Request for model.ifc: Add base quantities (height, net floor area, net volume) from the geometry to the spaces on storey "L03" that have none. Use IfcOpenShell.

First a look at what the model holds.

```python
import ifcopenshell
import ifcopenshell.util.element
import ifcopenshell.util.unit

model = ifcopenshell.open("model.ifc")
print(model.schema)
for unit_type in ("LENGTHUNIT", "AREAUNIT", "VOLUMEUNIT"):
    print(unit_type, ifcopenshell.util.unit.calculate_unit_scale(model, unit_type))
storey = next(s for s in model.by_type("IfcBuildingStorey") if s.Name == "L03")
spaces = [e for e in ifcopenshell.util.element.get_decomposition(storey) if e.is_a("IfcSpace")]
for e in sorted(spaces, key=lambda e: e.id()):
    print(e.id(), e.is_a(), e.Name, list(ifcopenshell.util.element.get_psets(e, qtos_only=True)), sep=" | ")
```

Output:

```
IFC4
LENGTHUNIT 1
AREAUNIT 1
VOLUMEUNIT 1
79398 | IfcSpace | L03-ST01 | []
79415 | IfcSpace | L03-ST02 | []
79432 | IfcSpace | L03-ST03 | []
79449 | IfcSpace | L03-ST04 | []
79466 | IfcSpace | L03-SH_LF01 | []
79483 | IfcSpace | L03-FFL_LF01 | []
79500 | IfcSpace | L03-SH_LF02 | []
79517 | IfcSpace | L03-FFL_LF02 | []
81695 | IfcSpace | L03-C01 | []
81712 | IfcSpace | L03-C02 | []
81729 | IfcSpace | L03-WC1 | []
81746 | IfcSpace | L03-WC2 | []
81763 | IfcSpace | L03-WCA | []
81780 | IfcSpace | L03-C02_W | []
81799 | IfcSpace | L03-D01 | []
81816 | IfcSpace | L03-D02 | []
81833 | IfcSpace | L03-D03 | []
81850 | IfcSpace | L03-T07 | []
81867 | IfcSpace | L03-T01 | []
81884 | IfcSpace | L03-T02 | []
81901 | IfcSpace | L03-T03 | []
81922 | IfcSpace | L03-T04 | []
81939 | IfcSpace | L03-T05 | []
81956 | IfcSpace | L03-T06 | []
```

```python
import ifcopenshell
import ifcopenshell.api.pset
import ifcopenshell.geom
import ifcopenshell.util.element
import ifcopenshell.util.shape
import ifcopenshell.util.unit

model = ifcopenshell.open("model.ifc")
unit_scale = ifcopenshell.util.unit.calculate_unit_scale(model)
area_scale = ifcopenshell.util.unit.calculate_unit_scale(model, "AREAUNIT")
volume_scale = ifcopenshell.util.unit.calculate_unit_scale(model, "VOLUMEUNIT")
settings = ifcopenshell.geom.settings()

storey = next(s for s in model.by_type("IfcBuildingStorey") if s.Name == "L03")
spaces = [e for e in ifcopenshell.util.element.get_decomposition(storey) if e.is_a("IfcSpace")]

for e in sorted(spaces, key=lambda e: e.id()):
    if ifcopenshell.util.element.get_psets(e, qtos_only=True, should_inherit=False):
        continue
    # Geometry comes back in metres, in the element's own axes.
    shape = ifcopenshell.geom.create_shape(settings, e)
    values = {
        "Height": ifcopenshell.util.shape.get_z(shape.geometry) / unit_scale,
        "NetFloorArea": ifcopenshell.util.shape.get_footprint_area(shape.geometry) / area_scale,
        "NetVolume": ifcopenshell.util.shape.get_volume(shape.geometry) / volume_scale,
    }
    qto = ifcopenshell.api.pset.add_qto(model, product=e, name="Qto_SpaceBaseQuantities")
    ifcopenshell.api.pset.edit_qto(model, qto=qto, properties=values)
    print(e.id(), {k: round(v, 3) for k, v in values.items()})

model.write("model_edited.ifc")
```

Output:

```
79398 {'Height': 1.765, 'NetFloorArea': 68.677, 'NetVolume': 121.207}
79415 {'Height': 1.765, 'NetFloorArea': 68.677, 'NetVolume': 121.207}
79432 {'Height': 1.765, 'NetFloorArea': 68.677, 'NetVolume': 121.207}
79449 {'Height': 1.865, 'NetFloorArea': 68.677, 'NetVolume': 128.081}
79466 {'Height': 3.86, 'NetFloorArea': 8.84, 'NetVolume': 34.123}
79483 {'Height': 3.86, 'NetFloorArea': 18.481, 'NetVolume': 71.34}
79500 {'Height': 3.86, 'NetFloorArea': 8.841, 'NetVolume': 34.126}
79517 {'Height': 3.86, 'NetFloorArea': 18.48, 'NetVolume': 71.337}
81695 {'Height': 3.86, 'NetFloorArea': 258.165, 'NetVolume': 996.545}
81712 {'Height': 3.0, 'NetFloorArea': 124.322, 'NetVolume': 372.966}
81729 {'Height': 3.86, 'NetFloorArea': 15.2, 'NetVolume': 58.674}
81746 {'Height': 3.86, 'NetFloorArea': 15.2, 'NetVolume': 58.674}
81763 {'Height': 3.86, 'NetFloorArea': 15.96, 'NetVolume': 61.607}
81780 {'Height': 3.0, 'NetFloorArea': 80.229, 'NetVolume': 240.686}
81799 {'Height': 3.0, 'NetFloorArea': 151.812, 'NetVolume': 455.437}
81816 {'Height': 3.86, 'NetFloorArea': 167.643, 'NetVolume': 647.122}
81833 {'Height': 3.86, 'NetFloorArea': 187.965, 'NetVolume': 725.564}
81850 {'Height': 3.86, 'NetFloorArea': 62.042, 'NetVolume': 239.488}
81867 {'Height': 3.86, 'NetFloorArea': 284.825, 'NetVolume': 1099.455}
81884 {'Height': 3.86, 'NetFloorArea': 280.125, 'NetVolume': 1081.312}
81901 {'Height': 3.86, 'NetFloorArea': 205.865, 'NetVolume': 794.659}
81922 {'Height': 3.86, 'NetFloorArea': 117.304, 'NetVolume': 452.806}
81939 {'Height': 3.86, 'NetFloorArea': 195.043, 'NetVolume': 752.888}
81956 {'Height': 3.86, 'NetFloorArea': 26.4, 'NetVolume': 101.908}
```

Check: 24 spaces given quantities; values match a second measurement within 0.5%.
